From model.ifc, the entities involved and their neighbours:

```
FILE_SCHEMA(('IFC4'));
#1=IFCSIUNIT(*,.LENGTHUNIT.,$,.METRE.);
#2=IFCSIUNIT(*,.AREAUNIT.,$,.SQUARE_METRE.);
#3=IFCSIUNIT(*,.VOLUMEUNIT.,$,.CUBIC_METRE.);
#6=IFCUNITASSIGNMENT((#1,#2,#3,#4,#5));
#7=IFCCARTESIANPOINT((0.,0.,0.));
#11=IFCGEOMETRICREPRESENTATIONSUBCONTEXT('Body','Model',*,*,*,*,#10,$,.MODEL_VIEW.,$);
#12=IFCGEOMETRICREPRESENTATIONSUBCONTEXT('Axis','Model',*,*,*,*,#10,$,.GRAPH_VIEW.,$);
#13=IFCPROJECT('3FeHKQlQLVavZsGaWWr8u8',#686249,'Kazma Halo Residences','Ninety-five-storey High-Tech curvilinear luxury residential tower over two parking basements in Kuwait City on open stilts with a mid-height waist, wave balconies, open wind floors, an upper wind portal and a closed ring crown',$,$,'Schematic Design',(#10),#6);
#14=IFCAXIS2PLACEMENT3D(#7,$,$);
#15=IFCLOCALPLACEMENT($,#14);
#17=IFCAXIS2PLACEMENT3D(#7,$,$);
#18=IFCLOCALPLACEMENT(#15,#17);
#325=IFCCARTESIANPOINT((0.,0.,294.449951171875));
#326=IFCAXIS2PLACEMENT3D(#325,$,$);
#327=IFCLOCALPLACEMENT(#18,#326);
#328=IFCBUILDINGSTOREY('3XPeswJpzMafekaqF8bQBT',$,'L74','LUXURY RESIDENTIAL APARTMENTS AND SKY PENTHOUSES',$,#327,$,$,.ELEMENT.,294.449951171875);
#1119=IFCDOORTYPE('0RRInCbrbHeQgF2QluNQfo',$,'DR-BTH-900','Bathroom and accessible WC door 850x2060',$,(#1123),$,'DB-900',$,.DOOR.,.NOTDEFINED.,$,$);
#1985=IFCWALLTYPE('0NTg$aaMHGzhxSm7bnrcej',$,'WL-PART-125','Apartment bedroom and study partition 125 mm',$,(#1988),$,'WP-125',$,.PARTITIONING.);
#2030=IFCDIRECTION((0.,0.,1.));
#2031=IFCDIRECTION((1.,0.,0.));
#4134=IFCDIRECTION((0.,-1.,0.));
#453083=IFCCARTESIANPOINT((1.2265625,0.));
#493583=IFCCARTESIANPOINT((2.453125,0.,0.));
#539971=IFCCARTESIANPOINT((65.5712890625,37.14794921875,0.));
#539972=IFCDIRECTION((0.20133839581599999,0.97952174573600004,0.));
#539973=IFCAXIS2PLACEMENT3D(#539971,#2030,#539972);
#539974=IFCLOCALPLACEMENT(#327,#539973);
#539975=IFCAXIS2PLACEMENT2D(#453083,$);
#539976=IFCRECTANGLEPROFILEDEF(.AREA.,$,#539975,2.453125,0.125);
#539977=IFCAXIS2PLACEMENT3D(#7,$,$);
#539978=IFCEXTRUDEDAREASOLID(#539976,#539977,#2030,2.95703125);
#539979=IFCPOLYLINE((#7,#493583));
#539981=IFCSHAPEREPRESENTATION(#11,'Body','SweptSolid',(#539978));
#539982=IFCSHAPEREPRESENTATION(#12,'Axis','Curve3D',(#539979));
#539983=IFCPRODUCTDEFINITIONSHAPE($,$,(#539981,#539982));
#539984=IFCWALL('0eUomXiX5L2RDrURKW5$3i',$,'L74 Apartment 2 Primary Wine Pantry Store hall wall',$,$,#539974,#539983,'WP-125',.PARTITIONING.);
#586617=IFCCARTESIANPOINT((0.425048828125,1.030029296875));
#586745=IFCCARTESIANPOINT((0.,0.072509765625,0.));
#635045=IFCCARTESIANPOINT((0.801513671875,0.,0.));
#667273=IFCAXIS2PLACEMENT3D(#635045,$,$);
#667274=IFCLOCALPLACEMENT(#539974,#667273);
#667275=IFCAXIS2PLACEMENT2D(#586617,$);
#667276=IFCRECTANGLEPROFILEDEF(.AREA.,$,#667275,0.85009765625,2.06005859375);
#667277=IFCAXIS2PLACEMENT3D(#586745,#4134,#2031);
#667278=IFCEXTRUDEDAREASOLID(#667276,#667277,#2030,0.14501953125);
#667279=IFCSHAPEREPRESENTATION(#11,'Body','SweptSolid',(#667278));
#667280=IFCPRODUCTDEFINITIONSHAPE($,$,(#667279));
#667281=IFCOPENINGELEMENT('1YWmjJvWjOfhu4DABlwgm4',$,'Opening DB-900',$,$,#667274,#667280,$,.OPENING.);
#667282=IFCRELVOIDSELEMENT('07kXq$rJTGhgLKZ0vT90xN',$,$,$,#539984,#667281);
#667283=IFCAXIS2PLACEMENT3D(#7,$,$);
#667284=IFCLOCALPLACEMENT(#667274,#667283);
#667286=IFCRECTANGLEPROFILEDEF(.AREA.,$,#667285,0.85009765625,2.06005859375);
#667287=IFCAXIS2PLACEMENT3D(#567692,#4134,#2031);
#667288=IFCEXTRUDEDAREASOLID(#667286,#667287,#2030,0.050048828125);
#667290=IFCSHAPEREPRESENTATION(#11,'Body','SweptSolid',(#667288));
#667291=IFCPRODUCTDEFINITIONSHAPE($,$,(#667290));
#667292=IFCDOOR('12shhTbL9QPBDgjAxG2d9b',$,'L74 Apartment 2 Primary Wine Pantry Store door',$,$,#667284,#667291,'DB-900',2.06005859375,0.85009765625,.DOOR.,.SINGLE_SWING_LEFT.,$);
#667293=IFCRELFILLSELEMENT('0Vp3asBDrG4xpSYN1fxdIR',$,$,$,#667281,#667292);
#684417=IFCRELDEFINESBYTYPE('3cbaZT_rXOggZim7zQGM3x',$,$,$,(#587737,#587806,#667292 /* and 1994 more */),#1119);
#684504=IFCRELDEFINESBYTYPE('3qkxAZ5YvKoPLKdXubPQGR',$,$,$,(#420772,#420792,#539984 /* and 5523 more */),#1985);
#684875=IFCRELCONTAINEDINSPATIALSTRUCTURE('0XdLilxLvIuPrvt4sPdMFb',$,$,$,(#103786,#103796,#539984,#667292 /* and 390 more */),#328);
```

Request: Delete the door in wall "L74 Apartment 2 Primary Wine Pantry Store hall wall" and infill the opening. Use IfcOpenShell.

```python
import ifcopenshell
import ifcopenshell.api.feature
import ifcopenshell.api.root
import ifcopenshell.geom
import ifcopenshell.util.shape

model = ifcopenshell.open("model.ifc")
settings = ifcopenshell.geom.settings()


def volume(element):
    """Net volume in cubic metres, openings subtracted."""
    shape = ifcopenshell.geom.create_shape(settings, element)
    return ifcopenshell.util.shape.get_volume(shape.geometry)


door = model.by_guid("12shhTbL9QPBDgjAxG2d9b")
opening = door.FillsVoids[0].RelatingOpeningElement
wall = opening.VoidsElements[0].RelatingBuildingElement
before = volume(wall)

ifcopenshell.api.root.remove_product(model, product=door)
ifcopenshell.api.feature.remove_feature(model, feature=opening)

after = volume(wall)

print(f"wall volume {before:.3f} -> {after:.3f} m3")

model.write("model_v2.ifc")
```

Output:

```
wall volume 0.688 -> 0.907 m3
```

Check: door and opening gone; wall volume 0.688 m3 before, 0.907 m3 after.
